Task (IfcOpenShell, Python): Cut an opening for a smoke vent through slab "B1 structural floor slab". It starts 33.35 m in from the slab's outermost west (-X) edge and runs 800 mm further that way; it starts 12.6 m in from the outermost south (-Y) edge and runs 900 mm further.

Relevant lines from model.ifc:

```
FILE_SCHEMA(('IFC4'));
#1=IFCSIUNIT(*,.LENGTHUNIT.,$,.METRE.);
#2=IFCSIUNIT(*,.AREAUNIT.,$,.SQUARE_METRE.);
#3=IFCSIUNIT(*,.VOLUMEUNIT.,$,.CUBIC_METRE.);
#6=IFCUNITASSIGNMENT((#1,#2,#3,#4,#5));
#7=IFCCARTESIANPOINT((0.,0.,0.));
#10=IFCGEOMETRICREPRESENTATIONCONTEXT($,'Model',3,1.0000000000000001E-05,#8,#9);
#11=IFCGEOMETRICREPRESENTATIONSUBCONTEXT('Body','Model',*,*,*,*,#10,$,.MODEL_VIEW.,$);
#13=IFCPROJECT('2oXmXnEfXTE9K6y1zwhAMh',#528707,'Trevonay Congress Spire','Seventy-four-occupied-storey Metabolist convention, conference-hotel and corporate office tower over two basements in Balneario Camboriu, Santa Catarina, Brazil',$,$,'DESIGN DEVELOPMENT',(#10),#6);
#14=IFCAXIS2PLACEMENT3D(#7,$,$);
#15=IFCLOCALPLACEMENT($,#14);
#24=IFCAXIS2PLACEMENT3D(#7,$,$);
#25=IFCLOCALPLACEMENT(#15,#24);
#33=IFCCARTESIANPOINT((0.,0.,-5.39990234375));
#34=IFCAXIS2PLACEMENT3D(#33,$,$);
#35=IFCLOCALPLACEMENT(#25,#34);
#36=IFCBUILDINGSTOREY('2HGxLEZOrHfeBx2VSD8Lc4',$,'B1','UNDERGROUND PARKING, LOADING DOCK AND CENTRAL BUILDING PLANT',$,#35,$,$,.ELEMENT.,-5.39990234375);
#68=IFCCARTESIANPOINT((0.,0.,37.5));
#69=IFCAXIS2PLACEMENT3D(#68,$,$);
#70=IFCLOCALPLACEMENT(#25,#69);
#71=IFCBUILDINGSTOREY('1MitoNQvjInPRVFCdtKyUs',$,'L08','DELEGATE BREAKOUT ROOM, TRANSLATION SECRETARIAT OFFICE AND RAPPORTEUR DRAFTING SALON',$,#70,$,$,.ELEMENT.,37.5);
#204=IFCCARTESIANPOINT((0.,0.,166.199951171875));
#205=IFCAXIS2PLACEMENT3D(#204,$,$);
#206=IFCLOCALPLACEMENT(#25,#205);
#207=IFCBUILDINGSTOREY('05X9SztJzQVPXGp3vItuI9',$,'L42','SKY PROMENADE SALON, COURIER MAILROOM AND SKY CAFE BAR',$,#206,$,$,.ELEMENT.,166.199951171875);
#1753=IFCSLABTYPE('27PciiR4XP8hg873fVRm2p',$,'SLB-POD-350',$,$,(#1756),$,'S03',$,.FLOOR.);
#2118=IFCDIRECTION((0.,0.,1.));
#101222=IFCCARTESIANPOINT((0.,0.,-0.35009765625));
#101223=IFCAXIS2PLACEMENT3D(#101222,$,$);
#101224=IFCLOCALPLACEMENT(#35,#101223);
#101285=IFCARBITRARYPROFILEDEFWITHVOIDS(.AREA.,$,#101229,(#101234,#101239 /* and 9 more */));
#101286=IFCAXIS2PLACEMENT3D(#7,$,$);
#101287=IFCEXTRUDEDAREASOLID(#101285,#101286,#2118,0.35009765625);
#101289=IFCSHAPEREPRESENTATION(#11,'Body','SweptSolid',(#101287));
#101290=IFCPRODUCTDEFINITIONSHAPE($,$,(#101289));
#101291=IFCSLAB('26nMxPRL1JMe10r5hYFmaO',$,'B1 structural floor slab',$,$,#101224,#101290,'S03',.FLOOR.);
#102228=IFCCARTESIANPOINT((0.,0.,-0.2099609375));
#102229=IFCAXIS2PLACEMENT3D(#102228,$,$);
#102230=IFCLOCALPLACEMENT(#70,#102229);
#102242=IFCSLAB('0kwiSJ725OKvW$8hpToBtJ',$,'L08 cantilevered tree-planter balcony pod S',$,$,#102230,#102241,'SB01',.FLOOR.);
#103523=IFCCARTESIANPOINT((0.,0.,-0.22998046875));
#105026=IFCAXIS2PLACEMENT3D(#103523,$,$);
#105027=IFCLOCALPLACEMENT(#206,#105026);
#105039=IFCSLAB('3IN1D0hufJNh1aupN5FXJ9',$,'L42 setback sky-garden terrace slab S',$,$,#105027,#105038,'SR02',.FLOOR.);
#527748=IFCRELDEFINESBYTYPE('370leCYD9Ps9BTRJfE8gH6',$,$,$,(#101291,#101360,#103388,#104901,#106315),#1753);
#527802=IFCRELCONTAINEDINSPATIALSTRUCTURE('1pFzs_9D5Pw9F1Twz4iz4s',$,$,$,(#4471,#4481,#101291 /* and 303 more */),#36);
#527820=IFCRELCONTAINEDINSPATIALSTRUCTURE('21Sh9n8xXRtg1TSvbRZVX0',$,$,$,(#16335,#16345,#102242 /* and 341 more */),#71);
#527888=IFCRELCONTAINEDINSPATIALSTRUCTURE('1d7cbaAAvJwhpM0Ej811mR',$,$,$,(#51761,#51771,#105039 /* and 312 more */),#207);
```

```python
import numpy as np
import ifcopenshell
import ifcopenshell.api.feature
import ifcopenshell.api.geometry
import ifcopenshell.api.root
import ifcopenshell.geom
import ifcopenshell.util.placement
import ifcopenshell.util.representation
import ifcopenshell.util.shape
import ifcopenshell.util.unit

model = ifcopenshell.open("model.ifc")
unit_scale = ifcopenshell.util.unit.calculate_unit_scale(model)
settings = ifcopenshell.geom.settings()


def volume(element):
    """Net volume in cubic metres, openings subtracted."""
    shape = ifcopenshell.geom.create_shape(settings, element)
    return ifcopenshell.util.shape.get_volume(shape.geometry)


slab = model.by_guid("26nMxPRL1JMe10r5hYFmaO")
before = volume(slab)

# Extent in the slab's own axes, in metres. The edges named are its -X and -Y sides.
slab_shape = ifcopenshell.geom.create_shape(settings, slab)
vertices = ifcopenshell.util.shape.get_vertices(slab_shape.geometry)
x_min, y_min, bottom = vertices.min(axis=0)
top = vertices[:, 2].max()

opening = ifcopenshell.api.root.create_entity(model, ifc_class="IfcOpeningElement", name="Smoke vent opening", predefined_type="OPENING")
context = ifcopenshell.util.representation.get_context(model, "Model", "Body", "MODEL_VIEW")
width, depth = 0.8, 0.9
outline = [(0.0, 0.0), (width, 0.0), (width, depth), (0.0, depth), (0.0, 0.0)]
# Overshoot both faces by 50 mm so the cut is clean.
shape = ifcopenshell.api.geometry.add_slab_representation(
    model, context=context, depth=top - bottom + 0.1, polyline=outline
)
ifcopenshell.api.geometry.assign_representation(model, product=opening, representation=shape)

matrix = ifcopenshell.util.placement.get_local_placement(slab.ObjectPlacement)
matrix[:, 3] = matrix @ np.append(np.array([x_min + 33.35, y_min + 12.6, bottom - 0.05]) / unit_scale, 1.0)
ifcopenshell.api.geometry.edit_object_placement(model, product=opening, matrix=matrix, is_si=False)
ifcopenshell.api.feature.add_feature(model, feature=opening, element=slab)

after = volume(slab)

print(f"slab volume {before:.3f} -> {after:.3f} m3")

model.write("model_rev.ifc")
```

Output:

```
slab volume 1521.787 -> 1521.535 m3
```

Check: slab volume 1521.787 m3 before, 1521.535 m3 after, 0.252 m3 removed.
